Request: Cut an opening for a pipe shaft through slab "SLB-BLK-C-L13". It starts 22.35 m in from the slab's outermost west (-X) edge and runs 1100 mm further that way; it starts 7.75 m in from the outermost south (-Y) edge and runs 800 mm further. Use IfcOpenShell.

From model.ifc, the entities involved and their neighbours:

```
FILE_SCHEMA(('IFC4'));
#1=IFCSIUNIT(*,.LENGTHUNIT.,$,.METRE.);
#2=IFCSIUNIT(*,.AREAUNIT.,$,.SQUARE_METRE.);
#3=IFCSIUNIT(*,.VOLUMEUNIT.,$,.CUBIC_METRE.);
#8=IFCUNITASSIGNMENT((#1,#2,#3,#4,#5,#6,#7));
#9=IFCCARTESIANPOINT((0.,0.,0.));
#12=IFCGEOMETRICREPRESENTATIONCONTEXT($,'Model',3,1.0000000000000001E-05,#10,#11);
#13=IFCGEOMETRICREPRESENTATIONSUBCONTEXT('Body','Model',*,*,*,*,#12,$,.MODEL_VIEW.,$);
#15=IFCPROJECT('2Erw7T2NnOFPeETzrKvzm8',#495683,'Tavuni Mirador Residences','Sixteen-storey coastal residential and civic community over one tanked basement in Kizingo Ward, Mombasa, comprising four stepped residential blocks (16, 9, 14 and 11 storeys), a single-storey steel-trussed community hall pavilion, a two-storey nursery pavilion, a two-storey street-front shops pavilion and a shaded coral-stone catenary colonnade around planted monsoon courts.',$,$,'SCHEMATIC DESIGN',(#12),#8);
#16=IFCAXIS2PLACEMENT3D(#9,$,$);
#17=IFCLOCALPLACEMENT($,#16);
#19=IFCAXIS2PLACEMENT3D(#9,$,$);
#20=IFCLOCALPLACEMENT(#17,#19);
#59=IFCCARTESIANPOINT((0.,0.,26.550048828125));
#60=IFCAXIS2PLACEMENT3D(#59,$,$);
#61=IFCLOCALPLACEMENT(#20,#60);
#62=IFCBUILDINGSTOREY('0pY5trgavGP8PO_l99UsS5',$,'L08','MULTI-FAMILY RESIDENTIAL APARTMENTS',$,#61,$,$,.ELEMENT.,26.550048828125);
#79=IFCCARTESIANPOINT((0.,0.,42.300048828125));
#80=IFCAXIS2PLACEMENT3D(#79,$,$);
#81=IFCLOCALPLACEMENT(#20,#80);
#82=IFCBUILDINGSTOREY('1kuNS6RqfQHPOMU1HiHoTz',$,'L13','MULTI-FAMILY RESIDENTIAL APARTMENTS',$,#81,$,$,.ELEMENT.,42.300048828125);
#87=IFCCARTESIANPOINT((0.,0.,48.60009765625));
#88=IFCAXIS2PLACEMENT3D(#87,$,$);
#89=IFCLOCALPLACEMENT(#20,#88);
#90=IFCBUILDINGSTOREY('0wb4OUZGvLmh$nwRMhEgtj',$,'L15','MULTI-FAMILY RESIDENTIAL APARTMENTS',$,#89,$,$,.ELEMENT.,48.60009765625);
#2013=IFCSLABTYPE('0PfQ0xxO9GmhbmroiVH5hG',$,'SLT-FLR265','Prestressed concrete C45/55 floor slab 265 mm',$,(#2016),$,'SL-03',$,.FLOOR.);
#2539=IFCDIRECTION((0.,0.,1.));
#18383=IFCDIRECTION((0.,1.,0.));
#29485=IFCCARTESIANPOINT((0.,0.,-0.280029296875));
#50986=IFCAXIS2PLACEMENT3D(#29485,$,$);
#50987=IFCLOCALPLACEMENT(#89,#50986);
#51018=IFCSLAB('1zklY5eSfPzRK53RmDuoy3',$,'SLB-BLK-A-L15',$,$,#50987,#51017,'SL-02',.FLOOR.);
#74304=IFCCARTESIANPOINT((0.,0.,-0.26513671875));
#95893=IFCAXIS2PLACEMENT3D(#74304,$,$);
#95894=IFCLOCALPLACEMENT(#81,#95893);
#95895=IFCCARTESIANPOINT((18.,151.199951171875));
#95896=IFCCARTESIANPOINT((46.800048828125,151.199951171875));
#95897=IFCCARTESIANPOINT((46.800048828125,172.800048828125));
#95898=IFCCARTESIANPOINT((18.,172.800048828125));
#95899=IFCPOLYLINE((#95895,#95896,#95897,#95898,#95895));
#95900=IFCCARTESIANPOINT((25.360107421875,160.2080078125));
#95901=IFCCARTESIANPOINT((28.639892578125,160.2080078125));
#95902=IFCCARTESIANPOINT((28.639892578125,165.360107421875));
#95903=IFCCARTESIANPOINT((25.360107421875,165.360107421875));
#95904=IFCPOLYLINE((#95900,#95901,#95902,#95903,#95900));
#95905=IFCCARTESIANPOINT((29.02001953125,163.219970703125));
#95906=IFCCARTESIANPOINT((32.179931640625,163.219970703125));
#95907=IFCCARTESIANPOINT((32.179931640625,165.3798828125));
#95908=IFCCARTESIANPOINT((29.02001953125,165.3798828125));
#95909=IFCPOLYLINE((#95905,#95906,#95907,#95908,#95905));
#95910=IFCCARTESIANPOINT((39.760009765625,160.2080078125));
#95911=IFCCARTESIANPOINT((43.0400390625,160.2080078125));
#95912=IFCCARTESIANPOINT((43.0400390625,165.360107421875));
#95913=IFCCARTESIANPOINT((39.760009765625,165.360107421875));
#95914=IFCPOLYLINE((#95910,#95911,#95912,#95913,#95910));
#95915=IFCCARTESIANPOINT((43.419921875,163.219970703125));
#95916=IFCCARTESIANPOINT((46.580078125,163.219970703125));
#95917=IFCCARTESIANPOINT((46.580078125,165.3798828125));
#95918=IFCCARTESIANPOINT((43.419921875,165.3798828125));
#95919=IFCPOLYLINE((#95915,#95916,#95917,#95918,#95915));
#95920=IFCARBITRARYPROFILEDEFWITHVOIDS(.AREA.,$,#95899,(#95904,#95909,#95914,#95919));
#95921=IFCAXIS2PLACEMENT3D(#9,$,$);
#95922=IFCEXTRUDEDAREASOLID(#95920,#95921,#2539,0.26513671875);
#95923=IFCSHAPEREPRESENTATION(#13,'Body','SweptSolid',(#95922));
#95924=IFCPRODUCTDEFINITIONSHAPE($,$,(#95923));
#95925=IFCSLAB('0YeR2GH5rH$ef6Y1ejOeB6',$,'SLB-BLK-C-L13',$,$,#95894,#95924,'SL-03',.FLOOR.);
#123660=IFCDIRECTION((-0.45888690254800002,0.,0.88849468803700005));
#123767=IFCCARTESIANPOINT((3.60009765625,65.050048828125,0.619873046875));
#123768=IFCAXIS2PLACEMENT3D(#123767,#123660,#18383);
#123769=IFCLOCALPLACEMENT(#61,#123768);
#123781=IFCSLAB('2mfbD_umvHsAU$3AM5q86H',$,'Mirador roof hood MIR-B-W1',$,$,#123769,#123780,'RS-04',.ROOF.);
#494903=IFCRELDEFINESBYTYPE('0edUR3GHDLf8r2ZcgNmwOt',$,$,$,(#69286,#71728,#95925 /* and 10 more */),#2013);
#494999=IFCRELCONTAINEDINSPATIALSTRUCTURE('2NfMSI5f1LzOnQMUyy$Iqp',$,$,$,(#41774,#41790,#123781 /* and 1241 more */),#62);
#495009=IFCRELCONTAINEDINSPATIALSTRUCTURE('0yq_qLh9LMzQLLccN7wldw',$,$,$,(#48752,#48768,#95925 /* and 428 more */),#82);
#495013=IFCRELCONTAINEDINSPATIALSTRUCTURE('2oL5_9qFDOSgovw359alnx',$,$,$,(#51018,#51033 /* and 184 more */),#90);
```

```python
import numpy as np
import ifcopenshell
import ifcopenshell.api.feature
import ifcopenshell.api.geometry
import ifcopenshell.api.root
import ifcopenshell.geom
import ifcopenshell.util.placement
import ifcopenshell.util.representation
import ifcopenshell.util.shape
import ifcopenshell.util.unit

model = ifcopenshell.open("model.ifc")
unit_scale = ifcopenshell.util.unit.calculate_unit_scale(model)
settings = ifcopenshell.geom.settings()


def volume(element):
    """Net volume in cubic metres, openings subtracted."""
    shape = ifcopenshell.geom.create_shape(settings, element)
    return ifcopenshell.util.shape.get_volume(shape.geometry)


slab = model.by_guid("0YeR2GH5rH$ef6Y1ejOeB6")
before = volume(slab)

# Extent in the slab's own axes, in metres. The edges named are its -X and -Y sides.
slab_shape = ifcopenshell.geom.create_shape(settings, slab)
vertices = ifcopenshell.util.shape.get_vertices(slab_shape.geometry)
x_min, y_min, bottom = vertices.min(axis=0)
top = vertices[:, 2].max()

opening = ifcopenshell.api.root.create_entity(model, ifc_class="IfcOpeningElement", name="Pipe shaft opening", predefined_type="OPENING")
context = ifcopenshell.util.representation.get_context(model, "Model", "Body", "MODEL_VIEW")
width, depth = 1.1, 0.8
outline = [(0.0, 0.0), (width, 0.0), (width, depth), (0.0, depth), (0.0, 0.0)]
# Overshoot both faces by 50 mm so the cut is clean.
shape = ifcopenshell.api.geometry.add_slab_representation(
    model, context=context, depth=top - bottom + 0.1, polyline=outline
)
ifcopenshell.api.geometry.assign_representation(model, product=opening, representation=shape)

matrix = ifcopenshell.util.placement.get_local_placement(slab.ObjectPlacement)
matrix[:, 3] = matrix @ np.append(np.array([x_min + 22.35, y_min + 7.75, bottom - 0.05]) / unit_scale, 1.0)
ifcopenshell.api.geometry.edit_object_placement(model, product=opening, matrix=matrix, is_si=False)
ifcopenshell.api.feature.add_feature(model, feature=opening, element=slab)

after = volume(slab)

print(f"slab volume {before:.3f} -> {after:.3f} m3")

model.write("model_v2.ifc")
```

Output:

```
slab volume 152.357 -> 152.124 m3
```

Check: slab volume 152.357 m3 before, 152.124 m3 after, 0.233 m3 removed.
